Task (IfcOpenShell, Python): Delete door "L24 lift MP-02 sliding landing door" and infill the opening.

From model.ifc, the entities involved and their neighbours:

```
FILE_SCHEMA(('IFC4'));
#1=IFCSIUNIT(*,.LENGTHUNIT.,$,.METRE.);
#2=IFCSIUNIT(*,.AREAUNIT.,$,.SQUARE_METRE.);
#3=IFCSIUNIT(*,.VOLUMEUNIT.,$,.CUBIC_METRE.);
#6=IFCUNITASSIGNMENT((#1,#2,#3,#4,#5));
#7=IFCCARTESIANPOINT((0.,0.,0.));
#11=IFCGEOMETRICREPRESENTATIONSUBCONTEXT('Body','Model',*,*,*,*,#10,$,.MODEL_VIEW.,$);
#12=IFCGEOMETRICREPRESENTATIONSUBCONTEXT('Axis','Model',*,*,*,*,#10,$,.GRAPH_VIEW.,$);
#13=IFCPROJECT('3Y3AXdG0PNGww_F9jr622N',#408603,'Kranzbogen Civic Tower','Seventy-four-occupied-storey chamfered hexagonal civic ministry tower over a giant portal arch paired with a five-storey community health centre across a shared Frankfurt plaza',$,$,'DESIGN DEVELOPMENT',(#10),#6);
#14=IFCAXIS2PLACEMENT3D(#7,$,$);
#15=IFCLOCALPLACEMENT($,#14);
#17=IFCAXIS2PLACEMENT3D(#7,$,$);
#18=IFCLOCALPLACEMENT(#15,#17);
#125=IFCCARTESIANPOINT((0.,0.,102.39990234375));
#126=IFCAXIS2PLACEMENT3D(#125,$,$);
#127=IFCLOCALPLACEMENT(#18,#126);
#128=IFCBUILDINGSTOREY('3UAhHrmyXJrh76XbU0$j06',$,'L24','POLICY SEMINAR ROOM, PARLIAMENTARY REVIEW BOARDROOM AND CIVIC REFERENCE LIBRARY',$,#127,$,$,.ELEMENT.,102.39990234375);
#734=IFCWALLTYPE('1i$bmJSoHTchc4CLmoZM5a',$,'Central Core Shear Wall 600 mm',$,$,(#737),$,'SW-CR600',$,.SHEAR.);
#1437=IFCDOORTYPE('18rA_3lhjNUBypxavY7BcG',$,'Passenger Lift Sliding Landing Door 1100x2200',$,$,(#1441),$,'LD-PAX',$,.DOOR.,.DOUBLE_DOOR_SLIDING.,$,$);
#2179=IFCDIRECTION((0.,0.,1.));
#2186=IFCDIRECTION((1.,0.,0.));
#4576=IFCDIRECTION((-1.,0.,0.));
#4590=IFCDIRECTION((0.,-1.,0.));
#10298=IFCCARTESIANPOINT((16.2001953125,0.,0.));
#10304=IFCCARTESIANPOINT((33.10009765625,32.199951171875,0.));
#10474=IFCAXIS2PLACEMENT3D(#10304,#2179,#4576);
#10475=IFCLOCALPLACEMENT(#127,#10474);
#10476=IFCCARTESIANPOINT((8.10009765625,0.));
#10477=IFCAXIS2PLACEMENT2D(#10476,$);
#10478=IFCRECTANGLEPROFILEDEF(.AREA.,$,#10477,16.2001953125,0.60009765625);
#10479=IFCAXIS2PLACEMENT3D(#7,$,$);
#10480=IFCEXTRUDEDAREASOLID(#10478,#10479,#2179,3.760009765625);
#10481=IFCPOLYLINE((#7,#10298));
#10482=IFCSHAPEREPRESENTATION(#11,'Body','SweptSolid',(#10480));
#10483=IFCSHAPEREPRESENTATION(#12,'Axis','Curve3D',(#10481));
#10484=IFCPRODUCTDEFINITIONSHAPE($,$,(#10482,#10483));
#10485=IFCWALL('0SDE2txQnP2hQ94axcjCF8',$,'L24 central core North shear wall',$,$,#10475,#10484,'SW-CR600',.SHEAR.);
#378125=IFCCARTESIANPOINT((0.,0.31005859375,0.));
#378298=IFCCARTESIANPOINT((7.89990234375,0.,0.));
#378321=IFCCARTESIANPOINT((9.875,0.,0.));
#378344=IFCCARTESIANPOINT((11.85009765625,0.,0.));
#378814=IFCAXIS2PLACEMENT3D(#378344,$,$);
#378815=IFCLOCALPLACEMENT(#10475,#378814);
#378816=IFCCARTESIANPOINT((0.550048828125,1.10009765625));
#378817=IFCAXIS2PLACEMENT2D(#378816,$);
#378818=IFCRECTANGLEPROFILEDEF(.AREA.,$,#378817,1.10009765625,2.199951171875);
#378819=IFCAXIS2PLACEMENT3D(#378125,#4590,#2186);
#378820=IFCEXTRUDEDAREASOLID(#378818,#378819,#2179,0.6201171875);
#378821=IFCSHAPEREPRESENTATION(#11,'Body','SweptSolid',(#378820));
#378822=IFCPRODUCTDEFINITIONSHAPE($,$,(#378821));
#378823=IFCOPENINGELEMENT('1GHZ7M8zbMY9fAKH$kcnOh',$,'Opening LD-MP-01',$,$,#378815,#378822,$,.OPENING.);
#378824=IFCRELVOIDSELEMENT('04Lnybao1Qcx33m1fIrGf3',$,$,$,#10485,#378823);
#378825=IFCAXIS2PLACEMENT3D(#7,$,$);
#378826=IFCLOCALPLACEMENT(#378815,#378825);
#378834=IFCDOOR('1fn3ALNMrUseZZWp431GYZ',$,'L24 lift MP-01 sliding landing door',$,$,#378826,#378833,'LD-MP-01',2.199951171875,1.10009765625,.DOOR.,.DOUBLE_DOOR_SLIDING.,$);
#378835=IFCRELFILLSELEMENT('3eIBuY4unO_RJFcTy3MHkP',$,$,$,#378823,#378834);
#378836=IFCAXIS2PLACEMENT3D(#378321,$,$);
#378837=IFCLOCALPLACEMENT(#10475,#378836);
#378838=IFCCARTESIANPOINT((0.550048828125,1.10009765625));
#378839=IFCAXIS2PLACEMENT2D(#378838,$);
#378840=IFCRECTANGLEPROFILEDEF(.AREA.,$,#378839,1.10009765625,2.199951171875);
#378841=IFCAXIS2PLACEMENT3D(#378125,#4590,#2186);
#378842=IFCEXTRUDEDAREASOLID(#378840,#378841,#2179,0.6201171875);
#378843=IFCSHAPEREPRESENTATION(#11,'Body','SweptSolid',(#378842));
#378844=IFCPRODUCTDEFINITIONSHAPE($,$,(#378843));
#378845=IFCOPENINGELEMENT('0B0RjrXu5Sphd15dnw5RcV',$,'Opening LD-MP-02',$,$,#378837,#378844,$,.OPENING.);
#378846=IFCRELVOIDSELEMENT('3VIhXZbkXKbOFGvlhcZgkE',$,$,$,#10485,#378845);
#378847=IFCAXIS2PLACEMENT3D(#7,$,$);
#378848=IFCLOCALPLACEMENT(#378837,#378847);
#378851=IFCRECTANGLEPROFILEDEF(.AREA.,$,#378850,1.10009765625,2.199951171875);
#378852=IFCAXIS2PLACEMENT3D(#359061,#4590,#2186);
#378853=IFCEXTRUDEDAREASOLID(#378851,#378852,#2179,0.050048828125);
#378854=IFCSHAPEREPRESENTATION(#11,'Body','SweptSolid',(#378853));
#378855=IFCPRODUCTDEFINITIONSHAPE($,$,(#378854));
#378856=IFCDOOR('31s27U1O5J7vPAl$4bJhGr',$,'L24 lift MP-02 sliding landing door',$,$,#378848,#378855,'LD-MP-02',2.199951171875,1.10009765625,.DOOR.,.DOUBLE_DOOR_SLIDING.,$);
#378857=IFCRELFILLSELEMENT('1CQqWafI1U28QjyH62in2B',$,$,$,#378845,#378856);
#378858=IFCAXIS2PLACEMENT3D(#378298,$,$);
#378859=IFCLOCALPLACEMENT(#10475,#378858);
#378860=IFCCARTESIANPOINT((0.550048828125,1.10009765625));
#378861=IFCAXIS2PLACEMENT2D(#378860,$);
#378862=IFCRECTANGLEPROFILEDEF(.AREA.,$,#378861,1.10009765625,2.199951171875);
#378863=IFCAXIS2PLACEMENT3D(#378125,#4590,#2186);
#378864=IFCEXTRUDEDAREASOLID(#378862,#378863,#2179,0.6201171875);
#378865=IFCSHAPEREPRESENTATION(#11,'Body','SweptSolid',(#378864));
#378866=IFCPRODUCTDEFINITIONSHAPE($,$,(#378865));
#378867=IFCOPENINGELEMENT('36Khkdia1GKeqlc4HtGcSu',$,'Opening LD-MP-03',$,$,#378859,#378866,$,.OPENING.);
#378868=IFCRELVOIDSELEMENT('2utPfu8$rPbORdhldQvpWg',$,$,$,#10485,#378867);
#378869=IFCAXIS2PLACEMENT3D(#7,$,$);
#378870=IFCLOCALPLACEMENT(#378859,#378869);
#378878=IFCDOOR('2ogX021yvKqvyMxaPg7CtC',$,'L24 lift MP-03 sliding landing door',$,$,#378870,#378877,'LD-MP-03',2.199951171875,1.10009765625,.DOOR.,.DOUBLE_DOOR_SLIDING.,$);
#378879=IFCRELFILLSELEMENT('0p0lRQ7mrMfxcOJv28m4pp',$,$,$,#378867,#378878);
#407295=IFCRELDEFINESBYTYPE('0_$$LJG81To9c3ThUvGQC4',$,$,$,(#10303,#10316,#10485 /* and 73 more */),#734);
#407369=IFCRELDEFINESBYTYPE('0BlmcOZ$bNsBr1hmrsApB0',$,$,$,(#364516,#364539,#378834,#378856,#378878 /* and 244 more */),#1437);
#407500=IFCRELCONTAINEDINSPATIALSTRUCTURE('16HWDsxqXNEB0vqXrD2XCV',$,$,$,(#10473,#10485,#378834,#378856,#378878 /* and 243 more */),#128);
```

```python
import ifcopenshell
import ifcopenshell.api.feature
import ifcopenshell.api.root
import ifcopenshell.geom
import ifcopenshell.util.shape

model = ifcopenshell.open("model.ifc")
settings = ifcopenshell.geom.settings()


def volume(element):
    """Net volume in cubic metres, openings subtracted."""
    shape = ifcopenshell.geom.create_shape(settings, element)
    return ifcopenshell.util.shape.get_volume(shape.geometry)


door = model.by_guid("31s27U1O5J7vPAl$4bJhGr")
opening = door.FillsVoids[0].RelatingOpeningElement
wall = opening.VoidsElements[0].RelatingBuildingElement
before = volume(wall)

ifcopenshell.api.root.remove_product(model, product=door)
ifcopenshell.api.feature.remove_feature(model, feature=opening)

after = volume(wall)

print(f"wall volume {before:.3f} -> {after:.3f} m3")

model.write("model_updated.ifc")
```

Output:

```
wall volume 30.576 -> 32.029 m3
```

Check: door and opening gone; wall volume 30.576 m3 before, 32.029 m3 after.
